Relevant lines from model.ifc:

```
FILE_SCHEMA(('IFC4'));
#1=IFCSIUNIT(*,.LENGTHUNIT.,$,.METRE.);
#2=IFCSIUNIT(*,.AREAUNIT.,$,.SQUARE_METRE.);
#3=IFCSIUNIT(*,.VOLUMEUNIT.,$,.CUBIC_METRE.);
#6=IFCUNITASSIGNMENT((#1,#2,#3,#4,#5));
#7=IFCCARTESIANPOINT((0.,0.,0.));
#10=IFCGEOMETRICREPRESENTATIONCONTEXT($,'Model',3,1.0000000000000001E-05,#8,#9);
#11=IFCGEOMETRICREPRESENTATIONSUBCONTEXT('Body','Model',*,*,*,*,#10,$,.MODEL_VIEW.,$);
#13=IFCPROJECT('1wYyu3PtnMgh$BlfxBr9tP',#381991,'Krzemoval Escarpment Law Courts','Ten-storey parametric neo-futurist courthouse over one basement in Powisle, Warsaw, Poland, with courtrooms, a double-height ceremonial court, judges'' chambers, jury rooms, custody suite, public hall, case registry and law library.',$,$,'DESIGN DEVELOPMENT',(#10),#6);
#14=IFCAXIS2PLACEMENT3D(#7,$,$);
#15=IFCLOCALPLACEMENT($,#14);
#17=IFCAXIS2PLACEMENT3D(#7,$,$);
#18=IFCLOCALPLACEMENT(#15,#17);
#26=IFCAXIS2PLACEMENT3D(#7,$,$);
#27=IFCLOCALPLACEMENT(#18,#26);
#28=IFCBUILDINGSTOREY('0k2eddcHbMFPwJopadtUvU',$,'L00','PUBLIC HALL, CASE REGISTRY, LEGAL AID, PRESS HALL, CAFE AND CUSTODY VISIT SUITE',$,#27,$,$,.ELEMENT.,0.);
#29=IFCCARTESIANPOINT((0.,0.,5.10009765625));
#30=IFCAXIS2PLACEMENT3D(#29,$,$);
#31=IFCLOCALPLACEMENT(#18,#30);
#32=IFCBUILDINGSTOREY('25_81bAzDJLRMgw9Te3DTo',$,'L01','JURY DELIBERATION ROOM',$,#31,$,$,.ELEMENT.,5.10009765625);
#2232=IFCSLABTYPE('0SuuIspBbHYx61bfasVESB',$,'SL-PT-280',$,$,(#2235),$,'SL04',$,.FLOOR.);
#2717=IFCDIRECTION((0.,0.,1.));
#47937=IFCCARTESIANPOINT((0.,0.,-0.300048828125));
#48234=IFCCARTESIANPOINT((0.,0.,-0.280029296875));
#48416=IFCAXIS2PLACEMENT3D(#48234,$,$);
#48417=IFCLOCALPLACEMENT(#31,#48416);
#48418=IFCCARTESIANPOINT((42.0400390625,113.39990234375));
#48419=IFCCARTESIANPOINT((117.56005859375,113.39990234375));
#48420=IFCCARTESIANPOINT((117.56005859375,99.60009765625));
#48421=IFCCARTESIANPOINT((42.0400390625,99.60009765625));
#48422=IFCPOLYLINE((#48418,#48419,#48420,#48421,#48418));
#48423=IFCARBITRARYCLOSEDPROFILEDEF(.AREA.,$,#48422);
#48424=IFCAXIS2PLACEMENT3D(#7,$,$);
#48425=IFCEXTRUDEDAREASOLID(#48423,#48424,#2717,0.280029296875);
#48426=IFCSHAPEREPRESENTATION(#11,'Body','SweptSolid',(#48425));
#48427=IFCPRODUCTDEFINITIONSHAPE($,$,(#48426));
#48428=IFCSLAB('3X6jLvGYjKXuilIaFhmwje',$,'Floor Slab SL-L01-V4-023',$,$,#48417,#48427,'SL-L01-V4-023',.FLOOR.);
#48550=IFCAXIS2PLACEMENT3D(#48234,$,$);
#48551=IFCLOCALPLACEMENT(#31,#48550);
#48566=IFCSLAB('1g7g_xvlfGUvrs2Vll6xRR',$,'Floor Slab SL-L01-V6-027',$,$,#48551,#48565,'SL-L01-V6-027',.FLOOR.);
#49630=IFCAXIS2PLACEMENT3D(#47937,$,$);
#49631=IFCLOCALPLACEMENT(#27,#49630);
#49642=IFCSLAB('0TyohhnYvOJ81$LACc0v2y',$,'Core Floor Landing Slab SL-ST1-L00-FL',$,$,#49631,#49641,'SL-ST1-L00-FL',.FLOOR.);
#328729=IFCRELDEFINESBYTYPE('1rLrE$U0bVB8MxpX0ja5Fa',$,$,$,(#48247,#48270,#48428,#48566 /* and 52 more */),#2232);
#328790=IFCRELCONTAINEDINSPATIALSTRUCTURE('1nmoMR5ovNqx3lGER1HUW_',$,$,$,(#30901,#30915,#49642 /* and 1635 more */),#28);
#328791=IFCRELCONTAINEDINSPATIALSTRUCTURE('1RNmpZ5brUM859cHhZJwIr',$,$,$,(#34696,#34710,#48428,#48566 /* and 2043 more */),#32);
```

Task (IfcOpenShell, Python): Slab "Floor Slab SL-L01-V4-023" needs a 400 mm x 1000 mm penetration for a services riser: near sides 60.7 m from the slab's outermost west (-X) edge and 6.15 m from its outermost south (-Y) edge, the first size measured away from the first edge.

```python
import numpy as np
import ifcopenshell
import ifcopenshell.api.feature
import ifcopenshell.api.geometry
import ifcopenshell.api.root
import ifcopenshell.geom
import ifcopenshell.util.placement
import ifcopenshell.util.representation
import ifcopenshell.util.shape
import ifcopenshell.util.unit

model = ifcopenshell.open("model.ifc")
unit_scale = ifcopenshell.util.unit.calculate_unit_scale(model)
settings = ifcopenshell.geom.settings()


def volume(element):
    """Net volume in cubic metres, openings subtracted."""
    shape = ifcopenshell.geom.create_shape(settings, element)
    return ifcopenshell.util.shape.get_volume(shape.geometry)


slab = model.by_guid("3X6jLvGYjKXuilIaFhmwje")
before = volume(slab)

# Extent in the slab's own axes, in metres. The edges named are its -X and -Y sides.
slab_shape = ifcopenshell.geom.create_shape(settings, slab)
vertices = ifcopenshell.util.shape.get_vertices(slab_shape.geometry)
x_min, y_min, bottom = vertices.min(axis=0)
top = vertices[:, 2].max()

opening = ifcopenshell.api.root.create_entity(model, ifc_class="IfcOpeningElement", name="Services riser opening", predefined_type="OPENING")
context = ifcopenshell.util.representation.get_context(model, "Model", "Body", "MODEL_VIEW")
width, depth = 0.4, 1
outline = [(0.0, 0.0), (width, 0.0), (width, depth), (0.0, depth), (0.0, 0.0)]
# Overshoot both faces by 50 mm so the cut is clean.
shape = ifcopenshell.api.geometry.add_slab_representation(
    model, context=context, depth=top - bottom + 0.1, polyline=outline
)
ifcopenshell.api.geometry.assign_representation(model, product=opening, representation=shape)

matrix = ifcopenshell.util.placement.get_local_placement(slab.ObjectPlacement)
matrix[:, 3] = matrix @ np.append(np.array([x_min + 60.7, y_min + 6.15, bottom - 0.05]) / unit_scale, 1.0)
ifcopenshell.api.geometry.edit_object_placement(model, product=opening, matrix=matrix, is_si=False)
ifcopenshell.api.feature.add_feature(model, feature=opening, element=slab)

after = volume(slab)

print(f"slab volume {before:.3f} -> {after:.3f} m3")

model.write("model-out.ifc")
```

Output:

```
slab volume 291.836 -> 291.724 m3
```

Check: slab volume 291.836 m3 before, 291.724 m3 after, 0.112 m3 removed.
